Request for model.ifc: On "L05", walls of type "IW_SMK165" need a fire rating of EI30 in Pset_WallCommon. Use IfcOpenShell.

First a look at what the model holds.

```python
import ifcopenshell
import ifcopenshell.util.element

model = ifcopenshell.open("model.ifc")
print(model.schema)
storey = next(s for s in model.by_type("IfcBuildingStorey") if s.Name == "L05")
walls = [e for e in ifcopenshell.util.element.get_decomposition(storey) if e.is_a("IfcWall")]
seen = {}
for e in walls:
    element_type = ifcopenshell.util.element.get_type(e)
    key = (element_type.Name if element_type != e and element_type else None, ifcopenshell.util.element.get_pset(e, "Pset_WallCommon", "FireRating"))
    seen[key] = seen.get(key, 0) + 1
for (name, value), count in sorted(seen.items(), key=str):
    print(count, "x", name, "|", value)
```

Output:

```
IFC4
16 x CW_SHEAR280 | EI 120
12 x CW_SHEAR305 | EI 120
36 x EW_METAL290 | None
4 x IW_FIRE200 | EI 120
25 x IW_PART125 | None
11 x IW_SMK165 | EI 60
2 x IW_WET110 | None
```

```python
import ifcopenshell
import ifcopenshell.api.pset
import ifcopenshell.util.element

model = ifcopenshell.open("model.ifc")

storey = next(s for s in model.by_type("IfcBuildingStorey") if s.Name == "L05")
walls = [e for e in ifcopenshell.util.element.get_decomposition(storey) if e.is_a("IfcWall")]

count = 0
for e in walls:
    element_type = ifcopenshell.util.element.get_type(e)
    if element_type in (None, e) or element_type.Name != "IW_SMK165":
        continue
    # add_pset returns the element's existing set when there is one.
    pset = ifcopenshell.api.pset.add_pset(model, product=e, name="Pset_WallCommon")
    ifcopenshell.api.pset.edit_pset(model, pset=pset, properties={"FireRating": "EI30"})
    count += 1

print(count, "walls updated")

model.write("model_v2.ifc")
```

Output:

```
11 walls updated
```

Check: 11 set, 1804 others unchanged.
